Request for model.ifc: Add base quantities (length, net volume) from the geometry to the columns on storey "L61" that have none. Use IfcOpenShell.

First a look at what the model holds.

```python
import ifcopenshell
import ifcopenshell.util.element
import ifcopenshell.util.unit

model = ifcopenshell.open("model.ifc")
print(model.schema)
for unit_type in ("LENGTHUNIT", "AREAUNIT", "VOLUMEUNIT"):
    print(unit_type, ifcopenshell.util.unit.calculate_unit_scale(model, unit_type))
storey = next(s for s in model.by_type("IfcBuildingStorey") if s.Name == "L61")
columns = [e for e in ifcopenshell.util.element.get_decomposition(storey) if e.is_a("IfcColumn")]
for e in sorted(columns, key=lambda e: e.id()):
    print(e.id(), e.is_a(), e.Name, list(ifcopenshell.util.element.get_psets(e, qtos_only=True)), sep=" | ")
```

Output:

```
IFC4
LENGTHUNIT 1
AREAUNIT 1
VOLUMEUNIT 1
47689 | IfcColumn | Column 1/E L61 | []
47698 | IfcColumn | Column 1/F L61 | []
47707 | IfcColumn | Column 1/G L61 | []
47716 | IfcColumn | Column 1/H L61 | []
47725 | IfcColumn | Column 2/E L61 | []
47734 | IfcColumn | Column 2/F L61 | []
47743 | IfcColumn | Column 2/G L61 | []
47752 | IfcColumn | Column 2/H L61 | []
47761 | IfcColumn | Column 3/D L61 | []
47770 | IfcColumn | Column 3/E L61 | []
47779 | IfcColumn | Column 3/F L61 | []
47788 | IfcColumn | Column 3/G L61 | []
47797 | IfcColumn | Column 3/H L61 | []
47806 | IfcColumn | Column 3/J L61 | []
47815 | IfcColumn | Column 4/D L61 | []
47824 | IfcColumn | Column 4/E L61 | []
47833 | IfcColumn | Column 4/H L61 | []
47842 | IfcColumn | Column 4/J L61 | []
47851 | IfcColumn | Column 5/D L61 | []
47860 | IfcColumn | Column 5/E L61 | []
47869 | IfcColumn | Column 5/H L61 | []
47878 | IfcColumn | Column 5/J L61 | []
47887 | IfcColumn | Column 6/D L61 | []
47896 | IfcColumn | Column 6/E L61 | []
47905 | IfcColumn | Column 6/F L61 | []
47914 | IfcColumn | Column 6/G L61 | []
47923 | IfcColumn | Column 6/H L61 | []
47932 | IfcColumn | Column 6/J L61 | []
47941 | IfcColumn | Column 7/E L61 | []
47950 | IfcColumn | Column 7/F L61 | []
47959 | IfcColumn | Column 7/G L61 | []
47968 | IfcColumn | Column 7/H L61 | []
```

```python
import ifcopenshell
import ifcopenshell.api.pset
import ifcopenshell.geom
import ifcopenshell.util.element
import ifcopenshell.util.shape
import ifcopenshell.util.unit

model = ifcopenshell.open("model.ifc")
unit_scale = ifcopenshell.util.unit.calculate_unit_scale(model)
volume_scale = ifcopenshell.util.unit.calculate_unit_scale(model, "VOLUMEUNIT")
settings = ifcopenshell.geom.settings()

storey = next(s for s in model.by_type("IfcBuildingStorey") if s.Name == "L61")
columns = [e for e in ifcopenshell.util.element.get_decomposition(storey) if e.is_a("IfcColumn")]

for e in sorted(columns, key=lambda e: e.id()):
    if ifcopenshell.util.element.get_psets(e, qtos_only=True, should_inherit=False):
        continue
    # Geometry comes back in metres, in the element's own axes.
    shape = ifcopenshell.geom.create_shape(settings, e)
    values = {
        "Length": ifcopenshell.util.shape.get_z(shape.geometry) / unit_scale,
        "NetVolume": ifcopenshell.util.shape.get_volume(shape.geometry) / volume_scale,
    }
    qto = ifcopenshell.api.pset.add_qto(model, product=e, name="Qto_ColumnBaseQuantities")
    ifcopenshell.api.pset.edit_qto(model, qto=qto, properties=values)
    print(e.id(), {k: round(v, 3) for k, v in values.items()})

model.write("model_updated.ifc")
```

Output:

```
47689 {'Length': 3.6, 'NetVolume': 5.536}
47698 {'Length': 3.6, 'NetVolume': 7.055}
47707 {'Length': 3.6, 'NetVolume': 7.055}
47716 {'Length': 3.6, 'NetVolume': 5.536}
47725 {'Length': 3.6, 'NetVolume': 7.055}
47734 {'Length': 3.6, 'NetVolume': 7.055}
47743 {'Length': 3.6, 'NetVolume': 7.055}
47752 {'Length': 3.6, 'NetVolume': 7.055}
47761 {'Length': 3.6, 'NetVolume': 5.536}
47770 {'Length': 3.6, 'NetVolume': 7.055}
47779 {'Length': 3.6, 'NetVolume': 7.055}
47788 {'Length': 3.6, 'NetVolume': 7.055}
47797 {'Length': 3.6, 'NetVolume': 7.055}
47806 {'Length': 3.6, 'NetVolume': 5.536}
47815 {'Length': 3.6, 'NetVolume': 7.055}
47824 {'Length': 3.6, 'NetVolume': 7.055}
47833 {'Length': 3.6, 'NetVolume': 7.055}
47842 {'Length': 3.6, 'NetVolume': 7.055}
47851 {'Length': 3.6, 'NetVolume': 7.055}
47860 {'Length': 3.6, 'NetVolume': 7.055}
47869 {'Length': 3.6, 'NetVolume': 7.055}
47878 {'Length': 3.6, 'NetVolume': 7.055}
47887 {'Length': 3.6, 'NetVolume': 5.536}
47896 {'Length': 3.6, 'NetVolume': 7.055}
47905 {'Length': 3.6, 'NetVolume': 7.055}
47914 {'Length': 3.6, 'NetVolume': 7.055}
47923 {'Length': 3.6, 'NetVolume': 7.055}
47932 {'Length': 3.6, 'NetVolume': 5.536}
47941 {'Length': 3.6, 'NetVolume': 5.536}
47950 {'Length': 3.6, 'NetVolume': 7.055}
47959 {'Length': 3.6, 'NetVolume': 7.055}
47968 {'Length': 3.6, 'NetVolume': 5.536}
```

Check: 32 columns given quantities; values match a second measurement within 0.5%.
